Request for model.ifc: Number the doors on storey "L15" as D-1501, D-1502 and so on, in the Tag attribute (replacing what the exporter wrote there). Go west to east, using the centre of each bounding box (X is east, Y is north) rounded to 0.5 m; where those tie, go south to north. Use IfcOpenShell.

First a look at what the model holds.

```python
import ifcopenshell
import ifcopenshell.util.element
import ifcopenshell.util.placement

model = ifcopenshell.open("model.ifc")
print(model.schema)
storey = next(s for s in model.by_type("IfcBuildingStorey") if s.Name == "L15")
doors = [e for e in ifcopenshell.util.element.get_decomposition(storey) if e.is_a("IfcDoor")]
for e in sorted(doors, key=lambda e: e.id()):
    origin = ifcopenshell.util.placement.get_local_placement(e.ObjectPlacement)[:3, 3]
    print(e.id(), e.Tag, e.Name, origin.round(2) + 0.0, sep=" | ")
```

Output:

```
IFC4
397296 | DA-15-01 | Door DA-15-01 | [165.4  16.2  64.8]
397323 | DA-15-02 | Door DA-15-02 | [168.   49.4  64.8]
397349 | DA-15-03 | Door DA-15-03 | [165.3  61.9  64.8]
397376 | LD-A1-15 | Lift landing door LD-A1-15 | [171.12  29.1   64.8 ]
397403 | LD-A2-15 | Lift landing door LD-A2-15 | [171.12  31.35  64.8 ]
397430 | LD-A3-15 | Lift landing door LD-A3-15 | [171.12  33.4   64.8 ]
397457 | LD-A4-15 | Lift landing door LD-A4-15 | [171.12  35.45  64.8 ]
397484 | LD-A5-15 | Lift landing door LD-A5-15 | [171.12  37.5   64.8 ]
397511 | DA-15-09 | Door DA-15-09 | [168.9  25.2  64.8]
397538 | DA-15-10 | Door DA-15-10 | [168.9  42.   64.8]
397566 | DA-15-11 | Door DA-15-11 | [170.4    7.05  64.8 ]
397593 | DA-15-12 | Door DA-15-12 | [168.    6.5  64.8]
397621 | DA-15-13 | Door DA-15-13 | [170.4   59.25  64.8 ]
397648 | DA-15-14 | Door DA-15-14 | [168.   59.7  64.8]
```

```python
import ifcopenshell
import ifcopenshell.geom
import ifcopenshell.util.element
import ifcopenshell.util.shape

model = ifcopenshell.open("model.ifc")
settings = ifcopenshell.geom.settings()
settings.set("use-world-coords", True)


def centre(element):
    shape = ifcopenshell.geom.create_shape(settings, element)
    return ifcopenshell.util.shape.get_bbox_centroid(shape.geometry)


storey = next(s for s in model.by_type("IfcBuildingStorey") if s.Name == "L15")
doors = [e for e in ifcopenshell.util.element.get_decomposition(storey) if e.is_a("IfcDoor")]

# Insertion points can sit at a corner or the storey origin, so sort by the geometry (in metres).
centres = {e: centre(e) for e in doors}
doors.sort(key=lambda e: (round(centres[e][0] / 0.5), centres[e][1]))

for i, e in enumerate(doors, start=1):
    number = f"D-15{i:02d}"
    e.Tag = number
    print(e.id(), number)

model.write("model_updated.ifc")
```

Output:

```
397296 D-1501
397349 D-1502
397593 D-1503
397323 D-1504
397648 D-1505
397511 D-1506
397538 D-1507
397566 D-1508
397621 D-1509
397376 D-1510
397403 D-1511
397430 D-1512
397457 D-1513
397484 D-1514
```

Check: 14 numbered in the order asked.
